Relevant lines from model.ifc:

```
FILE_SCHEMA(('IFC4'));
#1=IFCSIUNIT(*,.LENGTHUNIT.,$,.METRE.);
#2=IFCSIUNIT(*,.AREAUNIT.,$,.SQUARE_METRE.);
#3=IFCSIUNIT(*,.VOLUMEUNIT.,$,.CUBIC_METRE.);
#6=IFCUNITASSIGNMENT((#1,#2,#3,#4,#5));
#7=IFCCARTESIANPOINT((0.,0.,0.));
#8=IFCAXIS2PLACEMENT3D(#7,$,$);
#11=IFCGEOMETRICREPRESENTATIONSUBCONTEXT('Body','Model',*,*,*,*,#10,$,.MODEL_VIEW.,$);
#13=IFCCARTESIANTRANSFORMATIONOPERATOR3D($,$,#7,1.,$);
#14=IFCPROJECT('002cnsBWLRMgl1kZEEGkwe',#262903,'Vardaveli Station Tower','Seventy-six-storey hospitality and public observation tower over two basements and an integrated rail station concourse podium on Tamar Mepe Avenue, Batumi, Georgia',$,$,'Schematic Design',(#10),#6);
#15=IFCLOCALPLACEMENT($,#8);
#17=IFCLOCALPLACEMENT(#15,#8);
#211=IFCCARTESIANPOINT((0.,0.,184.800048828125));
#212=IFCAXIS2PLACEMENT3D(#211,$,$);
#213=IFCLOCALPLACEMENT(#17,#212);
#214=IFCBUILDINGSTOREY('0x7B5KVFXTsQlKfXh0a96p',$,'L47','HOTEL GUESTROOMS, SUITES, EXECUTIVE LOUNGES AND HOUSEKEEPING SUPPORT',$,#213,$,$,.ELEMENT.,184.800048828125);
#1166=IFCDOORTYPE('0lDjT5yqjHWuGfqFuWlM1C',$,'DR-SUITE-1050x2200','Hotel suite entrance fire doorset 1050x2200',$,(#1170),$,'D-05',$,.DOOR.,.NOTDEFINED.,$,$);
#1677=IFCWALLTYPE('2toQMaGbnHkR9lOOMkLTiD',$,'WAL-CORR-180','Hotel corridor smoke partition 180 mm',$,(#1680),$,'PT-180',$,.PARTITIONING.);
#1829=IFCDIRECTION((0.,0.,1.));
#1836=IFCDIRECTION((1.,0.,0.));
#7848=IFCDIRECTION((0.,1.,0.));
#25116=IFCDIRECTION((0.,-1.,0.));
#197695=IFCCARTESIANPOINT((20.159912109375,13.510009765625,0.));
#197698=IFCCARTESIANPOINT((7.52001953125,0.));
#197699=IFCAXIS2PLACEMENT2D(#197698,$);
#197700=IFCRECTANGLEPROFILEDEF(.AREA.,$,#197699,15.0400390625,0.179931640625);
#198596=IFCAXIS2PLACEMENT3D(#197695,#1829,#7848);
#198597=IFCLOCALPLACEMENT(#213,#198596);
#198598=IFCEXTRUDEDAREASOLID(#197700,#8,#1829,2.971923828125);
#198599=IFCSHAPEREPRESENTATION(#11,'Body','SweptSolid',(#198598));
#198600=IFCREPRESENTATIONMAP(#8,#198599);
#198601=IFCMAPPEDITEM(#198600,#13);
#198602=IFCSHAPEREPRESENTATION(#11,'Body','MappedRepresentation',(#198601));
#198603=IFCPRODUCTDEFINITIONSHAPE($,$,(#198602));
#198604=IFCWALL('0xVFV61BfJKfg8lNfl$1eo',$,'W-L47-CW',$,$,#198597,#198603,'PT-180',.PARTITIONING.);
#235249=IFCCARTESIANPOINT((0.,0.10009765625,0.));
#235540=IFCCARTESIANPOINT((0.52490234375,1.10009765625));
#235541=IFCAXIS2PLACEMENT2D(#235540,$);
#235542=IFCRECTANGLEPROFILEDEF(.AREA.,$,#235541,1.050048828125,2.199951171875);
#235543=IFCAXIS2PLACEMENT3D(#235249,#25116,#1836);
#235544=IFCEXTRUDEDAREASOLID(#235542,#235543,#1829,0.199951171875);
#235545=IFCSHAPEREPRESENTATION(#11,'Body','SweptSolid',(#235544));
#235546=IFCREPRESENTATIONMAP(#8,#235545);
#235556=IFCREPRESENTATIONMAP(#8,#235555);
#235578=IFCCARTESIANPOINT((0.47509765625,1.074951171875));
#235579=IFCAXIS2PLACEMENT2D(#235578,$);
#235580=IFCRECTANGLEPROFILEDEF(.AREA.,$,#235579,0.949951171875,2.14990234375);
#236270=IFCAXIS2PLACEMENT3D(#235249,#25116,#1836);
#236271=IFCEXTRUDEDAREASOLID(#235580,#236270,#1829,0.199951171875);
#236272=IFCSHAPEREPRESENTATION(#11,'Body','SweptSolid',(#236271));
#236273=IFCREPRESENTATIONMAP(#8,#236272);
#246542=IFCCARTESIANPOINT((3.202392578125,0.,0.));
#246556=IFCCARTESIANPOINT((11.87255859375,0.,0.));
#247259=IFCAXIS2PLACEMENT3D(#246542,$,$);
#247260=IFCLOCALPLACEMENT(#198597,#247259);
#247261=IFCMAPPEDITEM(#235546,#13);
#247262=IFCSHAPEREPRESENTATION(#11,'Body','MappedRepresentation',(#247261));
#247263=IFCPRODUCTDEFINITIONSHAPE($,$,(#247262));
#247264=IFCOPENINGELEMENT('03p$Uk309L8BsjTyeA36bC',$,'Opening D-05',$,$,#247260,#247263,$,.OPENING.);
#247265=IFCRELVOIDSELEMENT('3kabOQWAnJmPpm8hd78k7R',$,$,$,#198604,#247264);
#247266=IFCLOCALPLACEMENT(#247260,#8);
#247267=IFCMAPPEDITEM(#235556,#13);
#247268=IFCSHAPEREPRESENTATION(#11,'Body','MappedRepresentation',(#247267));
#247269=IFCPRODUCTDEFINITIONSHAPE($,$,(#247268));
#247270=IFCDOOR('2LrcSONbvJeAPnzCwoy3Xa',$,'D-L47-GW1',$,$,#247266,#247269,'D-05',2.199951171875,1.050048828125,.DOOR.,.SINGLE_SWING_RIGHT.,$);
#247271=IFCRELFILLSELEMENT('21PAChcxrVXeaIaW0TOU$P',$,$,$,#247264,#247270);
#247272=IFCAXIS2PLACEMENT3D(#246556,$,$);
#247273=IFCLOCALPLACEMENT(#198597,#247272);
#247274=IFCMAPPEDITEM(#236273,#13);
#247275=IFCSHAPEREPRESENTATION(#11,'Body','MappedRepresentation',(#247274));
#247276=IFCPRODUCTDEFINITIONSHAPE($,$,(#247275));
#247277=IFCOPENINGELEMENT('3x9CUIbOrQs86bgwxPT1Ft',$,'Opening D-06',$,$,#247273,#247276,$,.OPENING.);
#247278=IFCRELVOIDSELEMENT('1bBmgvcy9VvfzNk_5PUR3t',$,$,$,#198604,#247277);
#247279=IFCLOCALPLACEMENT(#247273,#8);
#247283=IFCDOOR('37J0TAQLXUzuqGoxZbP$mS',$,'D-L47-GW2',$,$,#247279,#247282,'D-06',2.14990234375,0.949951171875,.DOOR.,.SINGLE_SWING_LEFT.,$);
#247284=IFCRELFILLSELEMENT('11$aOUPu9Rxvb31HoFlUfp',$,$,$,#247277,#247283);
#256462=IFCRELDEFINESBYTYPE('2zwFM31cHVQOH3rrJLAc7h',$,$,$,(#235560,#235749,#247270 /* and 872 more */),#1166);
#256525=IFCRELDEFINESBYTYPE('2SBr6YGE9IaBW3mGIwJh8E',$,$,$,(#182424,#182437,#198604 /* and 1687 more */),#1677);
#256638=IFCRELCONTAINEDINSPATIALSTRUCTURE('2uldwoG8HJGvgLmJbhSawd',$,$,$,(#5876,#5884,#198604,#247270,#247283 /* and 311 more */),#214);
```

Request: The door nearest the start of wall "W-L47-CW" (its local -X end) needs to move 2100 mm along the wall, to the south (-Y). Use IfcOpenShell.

```python
import ifcopenshell
import ifcopenshell.api.geometry
import ifcopenshell.util.placement
import ifcopenshell.util.unit

model = ifcopenshell.open("model.ifc")
unit_scale = ifcopenshell.util.unit.calculate_unit_scale(model)

door = model.by_guid("2LrcSONbvJeAPnzCwoy3Xa")
opening = door.FillsVoids[0].RelatingOpeningElement
wall = opening.VoidsElements[0].RelatingBuildingElement

wall_matrix = ifcopenshell.util.placement.get_local_placement(wall.ObjectPlacement)
shift = wall_matrix[:3, 0] * -2.1 / unit_scale
before = ifcopenshell.util.placement.get_local_placement(door.ObjectPlacement)[:3, 3].copy()

# The door is placed relative to its opening, so it follows when the opening moves.
matrix = ifcopenshell.util.placement.get_local_placement(opening.ObjectPlacement)
matrix[:3, 3] += shift
ifcopenshell.api.geometry.edit_object_placement(
    model, product=opening, matrix=matrix, is_si=False, should_transform_children=True
)

after = ifcopenshell.util.placement.get_local_placement(door.ObjectPlacement)[:3, 3]
print("door moved by", (after - before).round(3) + 0.0)

model.write("model_edited.ifc")
```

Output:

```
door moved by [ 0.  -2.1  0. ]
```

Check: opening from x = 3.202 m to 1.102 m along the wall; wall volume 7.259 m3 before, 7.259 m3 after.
